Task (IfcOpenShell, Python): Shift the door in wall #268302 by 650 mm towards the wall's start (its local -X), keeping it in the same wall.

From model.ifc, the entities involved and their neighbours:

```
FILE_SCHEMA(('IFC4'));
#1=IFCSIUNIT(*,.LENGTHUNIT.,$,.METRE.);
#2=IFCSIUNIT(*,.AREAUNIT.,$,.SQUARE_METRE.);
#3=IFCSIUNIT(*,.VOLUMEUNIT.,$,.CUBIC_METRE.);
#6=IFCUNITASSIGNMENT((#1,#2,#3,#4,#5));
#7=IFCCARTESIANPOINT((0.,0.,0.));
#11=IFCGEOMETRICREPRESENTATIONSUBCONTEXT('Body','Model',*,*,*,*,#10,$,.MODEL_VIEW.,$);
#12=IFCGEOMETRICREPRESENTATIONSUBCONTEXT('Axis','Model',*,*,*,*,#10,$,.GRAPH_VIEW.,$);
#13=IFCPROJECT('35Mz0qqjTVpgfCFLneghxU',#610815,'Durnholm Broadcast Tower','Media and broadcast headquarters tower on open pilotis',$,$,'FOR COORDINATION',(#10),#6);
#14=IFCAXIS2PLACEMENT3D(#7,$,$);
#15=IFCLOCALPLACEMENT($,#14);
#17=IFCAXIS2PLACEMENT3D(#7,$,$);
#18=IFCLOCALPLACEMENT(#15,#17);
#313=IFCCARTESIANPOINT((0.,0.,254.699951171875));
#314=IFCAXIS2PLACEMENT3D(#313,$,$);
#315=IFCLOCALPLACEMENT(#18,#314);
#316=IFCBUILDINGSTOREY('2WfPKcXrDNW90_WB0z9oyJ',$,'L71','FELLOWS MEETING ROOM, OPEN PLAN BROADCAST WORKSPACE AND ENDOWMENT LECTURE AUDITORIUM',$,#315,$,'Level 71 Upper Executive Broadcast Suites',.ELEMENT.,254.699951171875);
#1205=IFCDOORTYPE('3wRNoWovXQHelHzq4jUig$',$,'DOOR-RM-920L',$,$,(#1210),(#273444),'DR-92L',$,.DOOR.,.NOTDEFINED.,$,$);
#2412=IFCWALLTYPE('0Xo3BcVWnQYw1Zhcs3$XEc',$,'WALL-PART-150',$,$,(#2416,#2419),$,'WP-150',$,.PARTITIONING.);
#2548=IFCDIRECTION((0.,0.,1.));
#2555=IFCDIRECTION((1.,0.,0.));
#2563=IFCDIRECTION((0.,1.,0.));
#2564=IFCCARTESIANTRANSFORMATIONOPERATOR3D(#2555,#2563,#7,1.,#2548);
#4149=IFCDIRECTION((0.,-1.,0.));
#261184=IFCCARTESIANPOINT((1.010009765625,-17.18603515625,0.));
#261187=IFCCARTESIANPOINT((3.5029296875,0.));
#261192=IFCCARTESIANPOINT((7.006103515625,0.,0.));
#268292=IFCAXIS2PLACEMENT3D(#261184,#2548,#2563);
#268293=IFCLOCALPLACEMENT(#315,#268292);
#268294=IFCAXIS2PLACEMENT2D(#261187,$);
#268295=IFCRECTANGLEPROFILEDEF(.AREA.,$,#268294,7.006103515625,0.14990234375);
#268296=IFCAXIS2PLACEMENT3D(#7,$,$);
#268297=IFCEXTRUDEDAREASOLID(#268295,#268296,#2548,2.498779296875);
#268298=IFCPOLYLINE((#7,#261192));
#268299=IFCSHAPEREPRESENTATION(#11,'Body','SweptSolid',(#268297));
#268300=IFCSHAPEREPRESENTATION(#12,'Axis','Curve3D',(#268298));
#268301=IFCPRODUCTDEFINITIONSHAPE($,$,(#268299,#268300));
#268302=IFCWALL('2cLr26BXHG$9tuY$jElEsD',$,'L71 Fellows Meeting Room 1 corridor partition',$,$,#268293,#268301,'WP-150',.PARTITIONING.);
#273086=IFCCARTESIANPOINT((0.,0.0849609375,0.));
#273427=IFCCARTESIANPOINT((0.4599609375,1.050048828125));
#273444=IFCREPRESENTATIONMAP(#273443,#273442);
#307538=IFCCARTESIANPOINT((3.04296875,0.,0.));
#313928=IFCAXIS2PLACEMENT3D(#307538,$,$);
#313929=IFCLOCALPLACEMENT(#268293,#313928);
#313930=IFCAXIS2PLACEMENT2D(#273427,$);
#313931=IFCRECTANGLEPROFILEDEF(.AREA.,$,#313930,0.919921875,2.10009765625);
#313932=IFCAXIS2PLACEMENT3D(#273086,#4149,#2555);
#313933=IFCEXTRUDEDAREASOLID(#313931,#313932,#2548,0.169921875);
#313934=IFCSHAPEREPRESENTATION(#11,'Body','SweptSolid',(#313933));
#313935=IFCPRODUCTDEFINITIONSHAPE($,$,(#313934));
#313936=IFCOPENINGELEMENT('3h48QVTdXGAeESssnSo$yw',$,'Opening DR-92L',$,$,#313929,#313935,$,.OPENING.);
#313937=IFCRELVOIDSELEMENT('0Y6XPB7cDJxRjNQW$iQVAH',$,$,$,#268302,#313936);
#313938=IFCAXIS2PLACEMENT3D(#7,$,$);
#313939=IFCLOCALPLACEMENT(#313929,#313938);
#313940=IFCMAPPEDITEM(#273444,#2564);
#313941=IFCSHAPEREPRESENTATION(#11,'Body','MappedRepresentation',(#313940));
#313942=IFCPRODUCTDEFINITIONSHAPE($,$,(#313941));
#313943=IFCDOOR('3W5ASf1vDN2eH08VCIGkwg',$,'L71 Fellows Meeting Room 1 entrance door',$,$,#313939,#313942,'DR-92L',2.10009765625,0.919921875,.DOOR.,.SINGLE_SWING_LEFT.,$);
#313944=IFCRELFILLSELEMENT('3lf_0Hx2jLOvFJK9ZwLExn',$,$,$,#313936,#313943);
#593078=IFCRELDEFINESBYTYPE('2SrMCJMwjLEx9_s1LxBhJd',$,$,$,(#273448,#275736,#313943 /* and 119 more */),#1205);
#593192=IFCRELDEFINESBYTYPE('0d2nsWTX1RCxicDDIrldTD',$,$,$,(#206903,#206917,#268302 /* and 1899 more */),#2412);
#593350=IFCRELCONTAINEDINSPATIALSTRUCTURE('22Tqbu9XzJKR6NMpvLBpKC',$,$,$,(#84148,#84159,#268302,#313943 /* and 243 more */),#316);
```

```python
import ifcopenshell
import ifcopenshell.api.geometry
import ifcopenshell.util.placement
import ifcopenshell.util.unit

model = ifcopenshell.open("model.ifc")
unit_scale = ifcopenshell.util.unit.calculate_unit_scale(model)

door = model.by_guid("3W5ASf1vDN2eH08VCIGkwg")
opening = door.FillsVoids[0].RelatingOpeningElement
wall = opening.VoidsElements[0].RelatingBuildingElement

wall_matrix = ifcopenshell.util.placement.get_local_placement(wall.ObjectPlacement)
shift = wall_matrix[:3, 0] * -0.65 / unit_scale
before = ifcopenshell.util.placement.get_local_placement(door.ObjectPlacement)[:3, 3].copy()

# The door is placed relative to its opening, so it follows when the opening moves.
matrix = ifcopenshell.util.placement.get_local_placement(opening.ObjectPlacement)
matrix[:3, 3] += shift
ifcopenshell.api.geometry.edit_object_placement(
    model, product=opening, matrix=matrix, is_si=False, should_transform_children=True
)

after = ifcopenshell.util.placement.get_local_placement(door.ObjectPlacement)[:3, 3]
print("door moved by", (after - before).round(3) + 0.0)

model.write("model_updated.ifc")
```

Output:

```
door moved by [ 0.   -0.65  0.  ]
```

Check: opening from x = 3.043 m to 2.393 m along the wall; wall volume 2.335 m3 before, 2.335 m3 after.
